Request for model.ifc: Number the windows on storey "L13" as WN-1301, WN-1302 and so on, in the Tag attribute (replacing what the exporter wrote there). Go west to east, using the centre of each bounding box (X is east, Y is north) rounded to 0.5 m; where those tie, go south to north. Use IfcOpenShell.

First a look at what the model holds.

```python
import ifcopenshell
import ifcopenshell.util.element
import ifcopenshell.util.placement

model = ifcopenshell.open("model.ifc")
print(model.schema)
storey = next(s for s in model.by_type("IfcBuildingStorey") if s.Name == "L13")
windows = [e for e in ifcopenshell.util.element.get_decomposition(storey) if e.is_a("IfcWindow")]
for e in sorted(windows, key=lambda e: e.id()):
    origin = ifcopenshell.util.placement.get_local_placement(e.ObjectPlacement)[:3, 3]
    print(e.id(), e.Tag, e.Name, origin.round(2) + 0.0, sep=" | ")
```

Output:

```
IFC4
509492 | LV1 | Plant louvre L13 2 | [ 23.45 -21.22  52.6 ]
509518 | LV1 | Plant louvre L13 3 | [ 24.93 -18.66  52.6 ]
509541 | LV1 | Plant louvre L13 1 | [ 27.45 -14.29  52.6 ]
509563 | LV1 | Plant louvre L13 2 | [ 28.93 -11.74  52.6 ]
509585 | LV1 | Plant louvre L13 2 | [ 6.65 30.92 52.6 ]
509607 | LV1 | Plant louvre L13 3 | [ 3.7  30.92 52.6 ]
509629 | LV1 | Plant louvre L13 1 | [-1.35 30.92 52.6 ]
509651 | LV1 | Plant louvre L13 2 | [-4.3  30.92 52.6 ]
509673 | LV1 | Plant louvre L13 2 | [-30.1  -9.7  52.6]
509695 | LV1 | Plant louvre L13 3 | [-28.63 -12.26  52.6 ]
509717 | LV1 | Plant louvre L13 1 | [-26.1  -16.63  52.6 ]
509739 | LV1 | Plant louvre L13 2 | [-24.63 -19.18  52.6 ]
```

```python
import ifcopenshell
import ifcopenshell.geom
import ifcopenshell.util.element
import ifcopenshell.util.shape

model = ifcopenshell.open("model.ifc")
settings = ifcopenshell.geom.settings()
settings.set("use-world-coords", True)


def centre(element):
    shape = ifcopenshell.geom.create_shape(settings, element)
    return ifcopenshell.util.shape.get_bbox_centroid(shape.geometry)


storey = next(s for s in model.by_type("IfcBuildingStorey") if s.Name == "L13")
windows = [e for e in ifcopenshell.util.element.get_decomposition(storey) if e.is_a("IfcWindow")]

# Insertion points can sit at a corner or the storey origin, so sort by the geometry (in metres).
centres = {e: centre(e) for e in windows}
windows.sort(key=lambda e: (round(centres[e][0] / 0.5), centres[e][1]))

for i, e in enumerate(windows, start=1):
    number = f"WN-13{i:02d}"
    e.Tag = number
    print(e.id(), number)

model.write("model_edited.ifc")
```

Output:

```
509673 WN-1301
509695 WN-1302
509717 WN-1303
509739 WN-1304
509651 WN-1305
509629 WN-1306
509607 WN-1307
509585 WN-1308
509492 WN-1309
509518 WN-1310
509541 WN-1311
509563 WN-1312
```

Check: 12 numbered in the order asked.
